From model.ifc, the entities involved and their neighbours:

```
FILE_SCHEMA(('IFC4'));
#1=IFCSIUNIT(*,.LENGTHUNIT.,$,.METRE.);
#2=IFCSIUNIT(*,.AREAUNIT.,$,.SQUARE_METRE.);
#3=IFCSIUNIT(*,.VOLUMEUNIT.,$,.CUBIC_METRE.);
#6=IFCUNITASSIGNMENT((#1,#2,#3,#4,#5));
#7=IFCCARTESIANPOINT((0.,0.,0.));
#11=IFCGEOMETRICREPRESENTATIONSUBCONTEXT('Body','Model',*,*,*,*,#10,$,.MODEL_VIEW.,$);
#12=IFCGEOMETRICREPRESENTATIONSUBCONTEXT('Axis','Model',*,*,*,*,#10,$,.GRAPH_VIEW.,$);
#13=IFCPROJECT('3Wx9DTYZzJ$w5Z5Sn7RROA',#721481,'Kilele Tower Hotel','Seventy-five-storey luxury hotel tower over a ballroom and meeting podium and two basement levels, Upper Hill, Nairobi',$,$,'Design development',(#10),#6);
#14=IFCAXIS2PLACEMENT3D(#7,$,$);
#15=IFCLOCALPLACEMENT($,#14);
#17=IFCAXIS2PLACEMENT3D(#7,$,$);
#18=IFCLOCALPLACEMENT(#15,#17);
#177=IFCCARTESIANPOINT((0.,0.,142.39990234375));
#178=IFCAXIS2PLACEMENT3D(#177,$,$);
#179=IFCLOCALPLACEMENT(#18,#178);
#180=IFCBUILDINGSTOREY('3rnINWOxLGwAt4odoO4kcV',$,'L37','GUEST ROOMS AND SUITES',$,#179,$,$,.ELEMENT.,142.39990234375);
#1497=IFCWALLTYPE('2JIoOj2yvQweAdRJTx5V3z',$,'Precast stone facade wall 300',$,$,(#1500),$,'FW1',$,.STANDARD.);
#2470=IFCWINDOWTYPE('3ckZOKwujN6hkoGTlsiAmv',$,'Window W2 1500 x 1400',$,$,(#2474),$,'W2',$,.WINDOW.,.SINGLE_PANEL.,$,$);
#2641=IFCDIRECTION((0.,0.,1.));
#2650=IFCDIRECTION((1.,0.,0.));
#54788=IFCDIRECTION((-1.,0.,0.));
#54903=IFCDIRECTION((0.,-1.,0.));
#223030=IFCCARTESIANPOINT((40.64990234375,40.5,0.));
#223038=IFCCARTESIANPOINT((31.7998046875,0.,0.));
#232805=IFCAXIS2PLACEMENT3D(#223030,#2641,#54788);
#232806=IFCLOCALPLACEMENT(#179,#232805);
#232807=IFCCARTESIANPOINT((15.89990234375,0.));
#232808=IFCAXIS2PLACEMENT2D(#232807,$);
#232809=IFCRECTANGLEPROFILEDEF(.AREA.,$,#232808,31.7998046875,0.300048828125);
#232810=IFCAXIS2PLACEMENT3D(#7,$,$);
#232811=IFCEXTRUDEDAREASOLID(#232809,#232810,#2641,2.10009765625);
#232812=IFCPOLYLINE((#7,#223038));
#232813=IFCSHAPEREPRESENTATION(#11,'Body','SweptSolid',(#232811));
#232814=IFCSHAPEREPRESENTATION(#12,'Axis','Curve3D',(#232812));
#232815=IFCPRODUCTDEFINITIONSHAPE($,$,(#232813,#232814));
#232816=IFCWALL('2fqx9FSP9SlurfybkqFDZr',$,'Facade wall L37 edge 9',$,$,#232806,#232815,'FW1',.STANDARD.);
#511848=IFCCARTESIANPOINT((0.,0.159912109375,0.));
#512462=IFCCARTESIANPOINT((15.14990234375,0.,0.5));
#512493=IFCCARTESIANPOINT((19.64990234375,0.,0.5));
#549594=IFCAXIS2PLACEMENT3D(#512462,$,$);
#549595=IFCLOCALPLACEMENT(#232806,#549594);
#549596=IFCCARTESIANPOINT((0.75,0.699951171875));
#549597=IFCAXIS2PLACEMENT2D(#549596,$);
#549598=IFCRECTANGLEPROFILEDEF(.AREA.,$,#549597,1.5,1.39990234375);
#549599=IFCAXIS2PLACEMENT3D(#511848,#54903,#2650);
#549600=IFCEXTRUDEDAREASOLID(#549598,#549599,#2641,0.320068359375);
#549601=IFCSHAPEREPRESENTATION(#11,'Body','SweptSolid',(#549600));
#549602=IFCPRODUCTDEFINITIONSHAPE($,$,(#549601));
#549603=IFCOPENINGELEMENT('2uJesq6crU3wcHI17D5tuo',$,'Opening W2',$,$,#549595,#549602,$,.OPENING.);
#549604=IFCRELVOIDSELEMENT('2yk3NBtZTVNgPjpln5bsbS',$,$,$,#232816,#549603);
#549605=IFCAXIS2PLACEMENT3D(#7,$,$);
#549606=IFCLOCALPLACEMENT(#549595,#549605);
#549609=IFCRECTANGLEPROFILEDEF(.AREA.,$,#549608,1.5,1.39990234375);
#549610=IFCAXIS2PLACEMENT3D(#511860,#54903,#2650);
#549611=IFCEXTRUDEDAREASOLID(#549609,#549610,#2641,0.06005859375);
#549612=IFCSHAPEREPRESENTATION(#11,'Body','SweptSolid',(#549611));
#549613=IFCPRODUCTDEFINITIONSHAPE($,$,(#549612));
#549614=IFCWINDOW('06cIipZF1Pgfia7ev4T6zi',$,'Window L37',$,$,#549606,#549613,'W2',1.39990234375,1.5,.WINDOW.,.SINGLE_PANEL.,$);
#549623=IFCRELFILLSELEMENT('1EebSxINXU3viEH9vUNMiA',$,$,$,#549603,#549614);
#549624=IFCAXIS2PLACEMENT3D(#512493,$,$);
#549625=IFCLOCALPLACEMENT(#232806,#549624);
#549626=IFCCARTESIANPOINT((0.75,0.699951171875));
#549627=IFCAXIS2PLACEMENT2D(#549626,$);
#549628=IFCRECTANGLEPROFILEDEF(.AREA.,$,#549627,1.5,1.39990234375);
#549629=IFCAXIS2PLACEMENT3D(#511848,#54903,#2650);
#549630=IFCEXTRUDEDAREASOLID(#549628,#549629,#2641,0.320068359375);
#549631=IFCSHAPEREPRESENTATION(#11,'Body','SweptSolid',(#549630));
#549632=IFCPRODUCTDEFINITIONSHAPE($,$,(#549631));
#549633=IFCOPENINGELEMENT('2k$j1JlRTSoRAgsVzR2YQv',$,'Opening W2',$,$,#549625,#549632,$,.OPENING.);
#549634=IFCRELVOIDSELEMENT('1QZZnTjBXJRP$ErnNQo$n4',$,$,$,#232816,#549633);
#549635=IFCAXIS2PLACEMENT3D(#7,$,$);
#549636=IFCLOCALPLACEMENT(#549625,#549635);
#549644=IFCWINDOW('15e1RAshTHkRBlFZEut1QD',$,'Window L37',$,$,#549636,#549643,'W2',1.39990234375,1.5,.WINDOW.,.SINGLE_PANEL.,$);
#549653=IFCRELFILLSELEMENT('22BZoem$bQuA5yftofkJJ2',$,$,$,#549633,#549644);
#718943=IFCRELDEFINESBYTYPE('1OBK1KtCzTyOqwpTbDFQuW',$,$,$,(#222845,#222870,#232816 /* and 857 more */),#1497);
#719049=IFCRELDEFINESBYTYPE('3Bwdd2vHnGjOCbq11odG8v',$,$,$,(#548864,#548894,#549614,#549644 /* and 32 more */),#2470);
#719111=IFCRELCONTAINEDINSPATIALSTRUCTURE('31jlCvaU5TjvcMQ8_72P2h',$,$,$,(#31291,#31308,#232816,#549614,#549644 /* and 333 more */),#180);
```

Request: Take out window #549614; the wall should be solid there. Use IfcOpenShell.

```python
import ifcopenshell
import ifcopenshell.api.feature
import ifcopenshell.api.root
import ifcopenshell.geom
import ifcopenshell.util.shape

model = ifcopenshell.open("model.ifc")
settings = ifcopenshell.geom.settings()


def volume(element):
    """Net volume in cubic metres, openings subtracted."""
    shape = ifcopenshell.geom.create_shape(settings, element)
    return ifcopenshell.util.shape.get_volume(shape.geometry)


window = model.by_id(549614)
opening = window.FillsVoids[0].RelatingOpeningElement
wall = opening.VoidsElements[0].RelatingBuildingElement
before = volume(wall)

ifcopenshell.api.root.remove_product(model, product=window)
ifcopenshell.api.feature.remove_feature(model, feature=opening)

after = volume(wall)

print(f"wall volume {before:.3f} -> {after:.3f} m3")

model.write("model_v2.ifc")
```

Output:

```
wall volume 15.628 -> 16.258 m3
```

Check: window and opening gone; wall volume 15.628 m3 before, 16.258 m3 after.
